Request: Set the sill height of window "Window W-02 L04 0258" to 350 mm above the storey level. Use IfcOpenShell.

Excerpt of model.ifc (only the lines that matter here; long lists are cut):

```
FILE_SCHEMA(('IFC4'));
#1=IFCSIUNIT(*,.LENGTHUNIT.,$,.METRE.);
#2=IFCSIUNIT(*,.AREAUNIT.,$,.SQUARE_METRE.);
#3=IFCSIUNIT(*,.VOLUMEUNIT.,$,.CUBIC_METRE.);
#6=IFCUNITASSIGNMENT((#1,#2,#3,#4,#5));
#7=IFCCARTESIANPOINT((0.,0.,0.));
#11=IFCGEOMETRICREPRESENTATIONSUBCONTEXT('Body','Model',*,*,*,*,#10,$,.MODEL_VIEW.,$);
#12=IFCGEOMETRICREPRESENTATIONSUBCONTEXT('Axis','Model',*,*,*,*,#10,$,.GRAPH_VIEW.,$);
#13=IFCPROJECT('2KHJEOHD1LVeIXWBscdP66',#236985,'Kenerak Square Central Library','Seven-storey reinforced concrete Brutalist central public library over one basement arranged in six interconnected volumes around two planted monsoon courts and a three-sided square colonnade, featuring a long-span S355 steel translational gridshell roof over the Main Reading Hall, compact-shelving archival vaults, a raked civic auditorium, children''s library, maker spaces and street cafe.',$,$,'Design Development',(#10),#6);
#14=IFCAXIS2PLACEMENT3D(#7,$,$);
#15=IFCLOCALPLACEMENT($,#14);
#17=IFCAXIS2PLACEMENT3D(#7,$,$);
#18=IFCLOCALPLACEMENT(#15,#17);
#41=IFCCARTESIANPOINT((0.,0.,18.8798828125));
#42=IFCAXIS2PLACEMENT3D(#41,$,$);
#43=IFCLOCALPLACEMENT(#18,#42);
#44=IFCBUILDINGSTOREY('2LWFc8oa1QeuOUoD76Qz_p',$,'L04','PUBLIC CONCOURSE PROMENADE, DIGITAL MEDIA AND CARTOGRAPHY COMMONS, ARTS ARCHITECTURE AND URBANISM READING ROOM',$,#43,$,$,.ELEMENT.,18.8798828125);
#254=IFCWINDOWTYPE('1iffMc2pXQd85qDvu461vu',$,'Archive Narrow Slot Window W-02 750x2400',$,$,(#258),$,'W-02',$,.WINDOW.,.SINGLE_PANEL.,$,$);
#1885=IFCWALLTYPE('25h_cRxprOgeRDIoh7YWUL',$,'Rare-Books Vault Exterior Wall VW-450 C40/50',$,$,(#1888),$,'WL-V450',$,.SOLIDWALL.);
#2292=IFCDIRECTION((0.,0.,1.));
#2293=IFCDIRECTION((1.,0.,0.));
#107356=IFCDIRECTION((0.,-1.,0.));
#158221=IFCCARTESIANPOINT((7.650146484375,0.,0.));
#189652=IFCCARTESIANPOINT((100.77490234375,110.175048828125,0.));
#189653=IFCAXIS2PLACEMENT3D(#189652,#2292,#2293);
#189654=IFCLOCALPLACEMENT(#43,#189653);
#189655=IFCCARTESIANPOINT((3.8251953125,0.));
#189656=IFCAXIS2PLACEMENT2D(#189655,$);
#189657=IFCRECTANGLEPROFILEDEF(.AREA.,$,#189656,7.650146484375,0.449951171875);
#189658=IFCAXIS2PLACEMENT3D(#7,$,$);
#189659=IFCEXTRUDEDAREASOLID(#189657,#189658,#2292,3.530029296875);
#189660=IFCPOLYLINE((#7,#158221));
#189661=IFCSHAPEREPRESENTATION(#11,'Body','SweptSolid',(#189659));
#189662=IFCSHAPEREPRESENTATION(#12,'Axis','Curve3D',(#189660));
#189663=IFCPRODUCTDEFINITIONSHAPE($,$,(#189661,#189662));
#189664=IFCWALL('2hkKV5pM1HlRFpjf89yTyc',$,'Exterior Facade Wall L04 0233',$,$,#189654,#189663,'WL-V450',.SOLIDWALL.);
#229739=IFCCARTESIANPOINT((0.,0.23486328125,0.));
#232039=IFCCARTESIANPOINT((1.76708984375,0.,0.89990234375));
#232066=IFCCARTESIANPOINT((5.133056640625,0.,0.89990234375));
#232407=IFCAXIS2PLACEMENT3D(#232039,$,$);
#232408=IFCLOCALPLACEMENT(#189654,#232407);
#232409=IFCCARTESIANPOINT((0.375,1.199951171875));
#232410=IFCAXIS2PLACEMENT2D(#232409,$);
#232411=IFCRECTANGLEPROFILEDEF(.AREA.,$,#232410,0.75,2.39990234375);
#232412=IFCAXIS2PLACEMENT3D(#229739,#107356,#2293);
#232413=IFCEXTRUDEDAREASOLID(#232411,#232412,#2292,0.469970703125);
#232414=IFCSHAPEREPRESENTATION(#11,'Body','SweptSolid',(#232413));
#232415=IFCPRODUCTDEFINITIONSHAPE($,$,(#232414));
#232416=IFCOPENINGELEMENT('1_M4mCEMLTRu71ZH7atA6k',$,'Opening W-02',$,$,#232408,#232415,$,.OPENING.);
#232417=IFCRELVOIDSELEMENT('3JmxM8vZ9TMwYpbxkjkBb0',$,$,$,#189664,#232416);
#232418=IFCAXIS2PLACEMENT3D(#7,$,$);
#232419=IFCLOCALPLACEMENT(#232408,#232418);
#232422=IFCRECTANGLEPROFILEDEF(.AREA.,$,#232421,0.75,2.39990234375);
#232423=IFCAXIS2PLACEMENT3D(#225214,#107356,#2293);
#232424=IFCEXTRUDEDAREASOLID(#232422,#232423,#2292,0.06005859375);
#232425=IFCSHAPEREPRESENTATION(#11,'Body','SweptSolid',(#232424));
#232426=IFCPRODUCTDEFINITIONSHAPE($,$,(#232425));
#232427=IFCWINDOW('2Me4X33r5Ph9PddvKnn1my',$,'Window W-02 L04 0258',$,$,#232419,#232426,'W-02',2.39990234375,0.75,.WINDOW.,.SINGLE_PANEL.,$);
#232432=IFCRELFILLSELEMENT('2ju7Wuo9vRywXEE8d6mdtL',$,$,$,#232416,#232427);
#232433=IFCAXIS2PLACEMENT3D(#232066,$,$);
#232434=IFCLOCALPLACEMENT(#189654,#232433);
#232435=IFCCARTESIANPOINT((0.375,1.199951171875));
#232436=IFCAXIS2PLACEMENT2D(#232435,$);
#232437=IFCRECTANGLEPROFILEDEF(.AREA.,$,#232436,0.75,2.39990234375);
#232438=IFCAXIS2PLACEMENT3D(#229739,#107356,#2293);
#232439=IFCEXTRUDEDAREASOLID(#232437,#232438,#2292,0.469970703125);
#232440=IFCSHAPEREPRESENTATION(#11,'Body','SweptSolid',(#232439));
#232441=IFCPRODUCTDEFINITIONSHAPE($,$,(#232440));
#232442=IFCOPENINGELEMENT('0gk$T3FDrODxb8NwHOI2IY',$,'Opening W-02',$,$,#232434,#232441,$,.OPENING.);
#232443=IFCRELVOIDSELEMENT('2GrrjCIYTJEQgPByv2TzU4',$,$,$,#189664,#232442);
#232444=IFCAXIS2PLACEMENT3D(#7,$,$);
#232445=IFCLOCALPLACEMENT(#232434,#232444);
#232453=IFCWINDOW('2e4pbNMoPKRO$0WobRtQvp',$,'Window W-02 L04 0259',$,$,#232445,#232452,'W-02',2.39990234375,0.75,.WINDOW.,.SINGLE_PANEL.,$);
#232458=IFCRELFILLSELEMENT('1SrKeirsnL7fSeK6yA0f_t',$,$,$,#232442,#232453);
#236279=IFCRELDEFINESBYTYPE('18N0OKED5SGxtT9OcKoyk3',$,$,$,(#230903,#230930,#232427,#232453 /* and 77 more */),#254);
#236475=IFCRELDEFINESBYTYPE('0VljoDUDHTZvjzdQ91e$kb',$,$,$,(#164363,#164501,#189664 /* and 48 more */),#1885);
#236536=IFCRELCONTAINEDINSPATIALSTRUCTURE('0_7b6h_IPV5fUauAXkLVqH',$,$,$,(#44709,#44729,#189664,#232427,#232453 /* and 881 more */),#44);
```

```python
import numpy as np
import ifcopenshell
import ifcopenshell.api.geometry
import ifcopenshell.geom
import ifcopenshell.util.element
import ifcopenshell.util.placement
import ifcopenshell.util.shape
import ifcopenshell.util.unit

model = ifcopenshell.open("model.ifc")
unit_scale = ifcopenshell.util.unit.calculate_unit_scale(model)

window = model.by_id(232427)
opening = window.FillsVoids[0].RelatingOpeningElement
storey = ifcopenshell.util.element.get_container(window, ifc_class="IfcBuildingStorey")
level = ifcopenshell.util.placement.get_local_placement(storey.ObjectPlacement)[2, 3]

# The opening's origin need not be at the sill, so measure its lowest point.
shape = ifcopenshell.geom.create_shape(ifcopenshell.geom.settings(), opening)
bottom = ifcopenshell.util.shape.get_shape_bottom_elevation(shape, shape.geometry) / unit_scale
dz = level + 0.35 / unit_scale - bottom

shift = np.array([0.0, 0.0, dz])
# The window is placed relative to its opening, so it follows when the opening moves.
matrix = ifcopenshell.util.placement.get_local_placement(opening.ObjectPlacement)
matrix[:3, 3] += shift
ifcopenshell.api.geometry.edit_object_placement(
    model, product=opening, matrix=matrix, is_si=False, should_transform_children=True
)

print(f"moved by {dz * unit_scale:+.3f} m")

model.write("model_updated.ifc")
```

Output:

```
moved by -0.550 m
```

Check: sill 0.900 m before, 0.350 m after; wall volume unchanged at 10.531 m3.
